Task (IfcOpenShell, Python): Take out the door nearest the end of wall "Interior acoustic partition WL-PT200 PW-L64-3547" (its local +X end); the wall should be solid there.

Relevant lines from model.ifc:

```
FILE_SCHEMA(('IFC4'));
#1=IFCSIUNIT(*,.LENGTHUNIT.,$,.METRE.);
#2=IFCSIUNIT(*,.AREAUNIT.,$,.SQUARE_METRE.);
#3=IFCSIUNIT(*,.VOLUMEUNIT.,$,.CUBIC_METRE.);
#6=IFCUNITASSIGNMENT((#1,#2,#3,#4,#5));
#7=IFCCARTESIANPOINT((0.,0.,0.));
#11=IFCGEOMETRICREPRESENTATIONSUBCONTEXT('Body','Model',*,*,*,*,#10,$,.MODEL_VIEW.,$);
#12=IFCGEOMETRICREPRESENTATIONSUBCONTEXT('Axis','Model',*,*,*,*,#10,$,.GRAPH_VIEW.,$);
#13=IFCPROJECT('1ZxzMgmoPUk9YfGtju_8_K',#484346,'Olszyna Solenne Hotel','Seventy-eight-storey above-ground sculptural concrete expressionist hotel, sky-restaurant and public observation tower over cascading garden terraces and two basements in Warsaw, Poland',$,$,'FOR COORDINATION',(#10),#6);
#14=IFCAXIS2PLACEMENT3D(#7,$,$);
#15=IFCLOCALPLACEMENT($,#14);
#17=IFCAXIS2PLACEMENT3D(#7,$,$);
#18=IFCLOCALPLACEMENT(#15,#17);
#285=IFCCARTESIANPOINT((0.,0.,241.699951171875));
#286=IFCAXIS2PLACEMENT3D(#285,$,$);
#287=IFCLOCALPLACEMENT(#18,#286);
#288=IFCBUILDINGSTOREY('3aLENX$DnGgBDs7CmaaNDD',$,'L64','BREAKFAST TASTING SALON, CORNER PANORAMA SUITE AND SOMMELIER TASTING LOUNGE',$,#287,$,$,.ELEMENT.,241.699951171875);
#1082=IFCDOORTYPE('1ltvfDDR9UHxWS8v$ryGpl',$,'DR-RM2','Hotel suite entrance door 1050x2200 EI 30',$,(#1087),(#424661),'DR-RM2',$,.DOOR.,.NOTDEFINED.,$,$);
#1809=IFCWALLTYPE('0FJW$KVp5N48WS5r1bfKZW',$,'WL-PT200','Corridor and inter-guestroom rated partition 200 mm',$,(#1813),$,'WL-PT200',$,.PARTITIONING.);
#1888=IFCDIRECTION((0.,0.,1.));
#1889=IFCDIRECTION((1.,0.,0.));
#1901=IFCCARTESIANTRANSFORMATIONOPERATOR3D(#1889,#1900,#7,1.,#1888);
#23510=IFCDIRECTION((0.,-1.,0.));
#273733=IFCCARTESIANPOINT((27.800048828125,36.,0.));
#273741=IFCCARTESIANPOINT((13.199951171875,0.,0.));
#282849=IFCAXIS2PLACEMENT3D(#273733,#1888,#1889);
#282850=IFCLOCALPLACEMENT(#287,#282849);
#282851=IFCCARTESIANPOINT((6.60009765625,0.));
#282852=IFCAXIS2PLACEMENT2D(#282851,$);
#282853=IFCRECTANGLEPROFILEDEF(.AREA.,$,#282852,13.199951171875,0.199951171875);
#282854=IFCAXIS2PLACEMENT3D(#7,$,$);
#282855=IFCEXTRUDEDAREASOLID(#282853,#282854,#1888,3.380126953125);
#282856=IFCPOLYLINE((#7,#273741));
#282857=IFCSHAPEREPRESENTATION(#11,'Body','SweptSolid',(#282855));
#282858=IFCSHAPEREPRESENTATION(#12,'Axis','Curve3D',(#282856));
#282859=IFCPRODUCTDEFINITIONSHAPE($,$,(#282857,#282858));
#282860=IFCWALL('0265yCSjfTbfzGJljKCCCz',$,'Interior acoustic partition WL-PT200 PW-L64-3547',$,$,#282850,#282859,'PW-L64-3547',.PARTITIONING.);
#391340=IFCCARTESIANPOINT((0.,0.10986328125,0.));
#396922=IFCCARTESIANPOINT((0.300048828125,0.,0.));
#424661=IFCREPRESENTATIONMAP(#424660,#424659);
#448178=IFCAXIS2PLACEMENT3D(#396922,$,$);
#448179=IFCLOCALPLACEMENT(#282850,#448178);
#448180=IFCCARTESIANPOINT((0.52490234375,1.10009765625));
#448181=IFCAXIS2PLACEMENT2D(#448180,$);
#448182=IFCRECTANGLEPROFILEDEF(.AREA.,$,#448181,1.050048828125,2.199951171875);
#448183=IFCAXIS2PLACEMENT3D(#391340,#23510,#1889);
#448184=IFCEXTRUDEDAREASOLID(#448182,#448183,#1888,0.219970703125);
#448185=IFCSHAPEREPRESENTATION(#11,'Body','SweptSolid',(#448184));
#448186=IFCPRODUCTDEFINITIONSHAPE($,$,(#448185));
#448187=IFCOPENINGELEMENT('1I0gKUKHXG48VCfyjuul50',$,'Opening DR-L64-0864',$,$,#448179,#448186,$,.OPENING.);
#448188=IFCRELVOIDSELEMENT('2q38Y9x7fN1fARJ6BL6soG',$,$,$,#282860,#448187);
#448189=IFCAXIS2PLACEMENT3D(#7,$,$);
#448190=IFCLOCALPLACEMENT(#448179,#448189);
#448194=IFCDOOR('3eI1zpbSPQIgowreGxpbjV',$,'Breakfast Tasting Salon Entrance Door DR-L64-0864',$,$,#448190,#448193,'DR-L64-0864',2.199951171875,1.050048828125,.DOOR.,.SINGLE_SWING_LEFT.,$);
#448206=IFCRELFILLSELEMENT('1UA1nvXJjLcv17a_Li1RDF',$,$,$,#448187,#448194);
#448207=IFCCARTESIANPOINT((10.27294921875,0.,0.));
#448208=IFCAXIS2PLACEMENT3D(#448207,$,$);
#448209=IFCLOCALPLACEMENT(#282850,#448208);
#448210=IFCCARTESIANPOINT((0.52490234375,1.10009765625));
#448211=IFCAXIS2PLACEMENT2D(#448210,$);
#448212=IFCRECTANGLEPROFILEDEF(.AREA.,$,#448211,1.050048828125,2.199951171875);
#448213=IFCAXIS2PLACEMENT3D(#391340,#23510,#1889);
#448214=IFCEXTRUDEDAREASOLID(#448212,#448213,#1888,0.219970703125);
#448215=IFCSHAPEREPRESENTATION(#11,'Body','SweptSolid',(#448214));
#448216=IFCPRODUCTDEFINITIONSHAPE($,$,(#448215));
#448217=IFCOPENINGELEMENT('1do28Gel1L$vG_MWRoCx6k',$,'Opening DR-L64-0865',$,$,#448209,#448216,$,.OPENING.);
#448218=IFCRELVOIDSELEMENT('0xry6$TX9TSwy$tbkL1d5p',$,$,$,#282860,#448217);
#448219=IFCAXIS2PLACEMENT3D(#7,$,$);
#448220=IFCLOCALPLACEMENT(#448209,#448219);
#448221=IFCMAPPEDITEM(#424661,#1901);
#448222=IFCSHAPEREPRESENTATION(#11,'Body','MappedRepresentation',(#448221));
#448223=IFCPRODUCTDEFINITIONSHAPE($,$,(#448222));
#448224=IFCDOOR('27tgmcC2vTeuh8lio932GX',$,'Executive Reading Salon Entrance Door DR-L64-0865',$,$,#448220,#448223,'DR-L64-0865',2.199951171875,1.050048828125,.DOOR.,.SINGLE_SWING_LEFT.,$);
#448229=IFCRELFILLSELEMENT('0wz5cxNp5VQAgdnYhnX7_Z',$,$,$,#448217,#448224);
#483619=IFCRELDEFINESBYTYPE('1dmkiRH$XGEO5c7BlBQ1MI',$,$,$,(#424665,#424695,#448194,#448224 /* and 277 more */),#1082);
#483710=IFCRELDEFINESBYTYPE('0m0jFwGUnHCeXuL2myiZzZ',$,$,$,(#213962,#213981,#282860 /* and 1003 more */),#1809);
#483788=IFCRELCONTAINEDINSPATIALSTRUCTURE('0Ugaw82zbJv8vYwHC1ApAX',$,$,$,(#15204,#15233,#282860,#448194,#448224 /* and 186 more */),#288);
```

```python
import ifcopenshell
import ifcopenshell.api.feature
import ifcopenshell.api.root
import ifcopenshell.geom
import ifcopenshell.util.shape

model = ifcopenshell.open("model.ifc")
settings = ifcopenshell.geom.settings()


def volume(element):
    """Net volume in cubic metres, openings subtracted."""
    shape = ifcopenshell.geom.create_shape(settings, element)
    return ifcopenshell.util.shape.get_volume(shape.geometry)


door = model.by_guid("27tgmcC2vTeuh8lio932GX")
opening = door.FillsVoids[0].RelatingOpeningElement
wall = opening.VoidsElements[0].RelatingBuildingElement
before = volume(wall)

ifcopenshell.api.root.remove_product(model, product=door)
ifcopenshell.api.feature.remove_feature(model, feature=opening)

after = volume(wall)

print(f"wall volume {before:.3f} -> {after:.3f} m3")

model.write("model_updated.ifc")
```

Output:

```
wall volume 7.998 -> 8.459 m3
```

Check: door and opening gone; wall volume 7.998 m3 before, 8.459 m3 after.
